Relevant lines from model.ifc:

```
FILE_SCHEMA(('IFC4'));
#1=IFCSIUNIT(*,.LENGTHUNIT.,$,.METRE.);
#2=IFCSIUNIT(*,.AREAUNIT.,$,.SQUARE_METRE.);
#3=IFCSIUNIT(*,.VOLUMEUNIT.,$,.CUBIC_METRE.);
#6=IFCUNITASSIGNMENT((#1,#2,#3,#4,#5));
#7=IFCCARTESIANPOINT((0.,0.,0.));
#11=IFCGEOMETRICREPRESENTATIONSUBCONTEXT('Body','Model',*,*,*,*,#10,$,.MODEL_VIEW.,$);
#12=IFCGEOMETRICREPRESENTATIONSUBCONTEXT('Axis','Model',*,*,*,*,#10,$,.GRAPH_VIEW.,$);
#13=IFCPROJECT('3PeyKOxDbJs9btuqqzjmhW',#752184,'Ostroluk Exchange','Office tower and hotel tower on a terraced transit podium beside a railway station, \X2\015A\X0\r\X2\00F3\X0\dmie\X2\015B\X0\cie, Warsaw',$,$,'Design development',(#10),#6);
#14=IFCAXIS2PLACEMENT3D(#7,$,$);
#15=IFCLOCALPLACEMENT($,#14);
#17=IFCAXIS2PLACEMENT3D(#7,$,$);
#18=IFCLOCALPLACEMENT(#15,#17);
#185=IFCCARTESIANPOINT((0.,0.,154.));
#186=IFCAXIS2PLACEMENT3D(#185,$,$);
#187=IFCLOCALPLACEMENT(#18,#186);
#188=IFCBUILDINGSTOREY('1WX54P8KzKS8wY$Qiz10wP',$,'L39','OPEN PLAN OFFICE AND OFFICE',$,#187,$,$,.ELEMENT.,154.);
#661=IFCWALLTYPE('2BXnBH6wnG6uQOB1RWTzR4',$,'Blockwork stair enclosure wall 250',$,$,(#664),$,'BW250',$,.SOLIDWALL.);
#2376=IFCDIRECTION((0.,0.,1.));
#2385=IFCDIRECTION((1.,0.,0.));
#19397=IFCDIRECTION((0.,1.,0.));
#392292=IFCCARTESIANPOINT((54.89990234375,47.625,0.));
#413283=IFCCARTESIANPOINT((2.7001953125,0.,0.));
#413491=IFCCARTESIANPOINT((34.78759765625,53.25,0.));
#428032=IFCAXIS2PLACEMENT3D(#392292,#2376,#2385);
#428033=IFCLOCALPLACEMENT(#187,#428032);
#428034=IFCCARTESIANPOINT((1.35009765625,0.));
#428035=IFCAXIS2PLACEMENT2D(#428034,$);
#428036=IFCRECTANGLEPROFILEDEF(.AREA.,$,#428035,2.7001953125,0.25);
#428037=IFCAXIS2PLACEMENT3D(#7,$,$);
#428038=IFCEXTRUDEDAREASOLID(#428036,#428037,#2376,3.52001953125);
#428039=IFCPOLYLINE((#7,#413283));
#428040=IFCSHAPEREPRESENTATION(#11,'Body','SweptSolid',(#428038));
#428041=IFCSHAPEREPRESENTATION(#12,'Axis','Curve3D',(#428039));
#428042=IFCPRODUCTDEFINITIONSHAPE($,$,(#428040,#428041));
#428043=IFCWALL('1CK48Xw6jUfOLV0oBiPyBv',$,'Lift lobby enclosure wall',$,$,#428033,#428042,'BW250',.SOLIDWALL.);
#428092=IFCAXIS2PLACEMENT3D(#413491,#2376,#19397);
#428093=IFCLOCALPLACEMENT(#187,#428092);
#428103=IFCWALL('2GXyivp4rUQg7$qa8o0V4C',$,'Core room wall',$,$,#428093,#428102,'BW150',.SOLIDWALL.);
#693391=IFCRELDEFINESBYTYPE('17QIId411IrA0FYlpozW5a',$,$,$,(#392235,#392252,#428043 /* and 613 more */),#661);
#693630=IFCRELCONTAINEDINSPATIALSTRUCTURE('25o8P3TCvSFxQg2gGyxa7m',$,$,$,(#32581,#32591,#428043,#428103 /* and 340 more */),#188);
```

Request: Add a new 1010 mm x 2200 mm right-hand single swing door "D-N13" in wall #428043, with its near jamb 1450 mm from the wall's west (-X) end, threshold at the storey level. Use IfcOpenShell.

```python
import numpy as np
import ifcopenshell
import ifcopenshell.api.feature
import ifcopenshell.api.geometry
import ifcopenshell.api.root
import ifcopenshell.api.spatial
import ifcopenshell.geom
import ifcopenshell.util.element
import ifcopenshell.util.placement
import ifcopenshell.util.representation
import ifcopenshell.util.shape
import ifcopenshell.util.unit

model = ifcopenshell.open("model.ifc")
unit_scale = ifcopenshell.util.unit.calculate_unit_scale(model)
settings = ifcopenshell.geom.settings()


def volume(element):
    """Net volume in cubic metres, openings subtracted."""
    shape = ifcopenshell.geom.create_shape(settings, element)
    return ifcopenshell.util.shape.get_volume(shape.geometry)


wall = model.by_id(428043)
storey = ifcopenshell.util.element.get_container(wall, ifc_class="IfcBuildingStorey")
context = ifcopenshell.util.representation.get_context(model, "Model", "Body", "MODEL_VIEW")
before = volume(wall)

width, height, from_end, sill = 1.01, 2.2, 1.45, 0.0  # metres

# The wall runs along its own X axis, and the end named is its -X end.
wall_shape = ifcopenshell.geom.create_shape(settings, wall)
x, y, z = ifcopenshell.util.shape.get_vertices(wall_shape.geometry).T
start = x.min() + from_end
face, thickness = float(y.min()), float(y.max() - y.min())
wall_matrix = ifcopenshell.util.placement.get_local_placement(wall.ObjectPlacement)
level = ifcopenshell.util.placement.get_local_placement(storey.ObjectPlacement)[2, 3]


def in_wall(x, y):
    """Placement at x, y metres in the wall's axes, at sill height."""
    matrix = wall_matrix.copy()
    matrix[:, 3] = wall_matrix @ np.array([x / unit_scale, y / unit_scale, 0.0, 1.0])
    matrix[2, 3] = level + sill / unit_scale
    return matrix


# Opening: a box that overshoots both wall faces by 50 mm.
opening = ifcopenshell.api.root.create_entity(model, ifc_class="IfcOpeningElement", predefined_type="OPENING")
box = ifcopenshell.api.geometry.add_wall_representation(
    model, context=context, length=width, height=height, thickness=thickness + 0.1
)
ifcopenshell.api.geometry.assign_representation(model, product=opening, representation=box)
ifcopenshell.api.geometry.edit_object_placement(model, product=opening, matrix=in_wall(start, face - 0.05), is_si=False)
ifcopenshell.api.feature.add_feature(model, feature=opening, element=wall)

door = ifcopenshell.api.root.create_entity(model, ifc_class="IfcDoor", name="D-N13", predefined_type="DOOR")
door.OverallWidth, door.OverallHeight = width / unit_scale, height / unit_scale
door.OperationType = "SINGLE_SWING_RIGHT"
body = ifcopenshell.api.geometry.add_door_representation(
    model,
    context=context,
    overall_width=door.OverallWidth,
    overall_height=door.OverallHeight,
    operation_type="SINGLE_SWING_RIGHT",
    lining_properties={"LiningDepth": thickness / unit_scale, "ThresholdDepth": thickness / unit_scale},
)
ifcopenshell.api.geometry.assign_representation(model, product=door, representation=body)
ifcopenshell.api.spatial.assign_container(model, products=[door], relating_structure=storey)
ifcopenshell.api.feature.add_filling(model, opening=opening, element=door)

# The lining spans the wall, so the door starts at the wall face.
ifcopenshell.api.geometry.edit_object_placement(model, product=door, matrix=in_wall(start, face), is_si=False)

after = volume(wall)

print(f"wall volume {before:.3f} -> {after:.3f} m3")

model.write("model_edited.ifc")
```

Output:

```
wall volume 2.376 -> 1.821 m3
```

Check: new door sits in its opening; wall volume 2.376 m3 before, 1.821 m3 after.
